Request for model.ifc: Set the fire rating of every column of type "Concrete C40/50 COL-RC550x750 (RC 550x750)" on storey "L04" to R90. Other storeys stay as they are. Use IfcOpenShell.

First a look at what the model holds.

```python
import ifcopenshell
import ifcopenshell.util.element

model = ifcopenshell.open("model.ifc")
print(model.schema)
storey = next(s for s in model.by_type("IfcBuildingStorey") if s.Name == "L04")
columns = [e for e in ifcopenshell.util.element.get_decomposition(storey) if e.is_a("IfcColumn")]
seen = {}
for e in columns:
    element_type = ifcopenshell.util.element.get_type(e)
    key = (element_type.Name if element_type != e and element_type else None, ifcopenshell.util.element.get_pset(e, "Pset_ColumnCommon", "FireRating"))
    seen[key] = seen.get(key, 0) + 1
for (name, value), count in sorted(seen.items(), key=str):
    print(count, "x", name, "|", value)
```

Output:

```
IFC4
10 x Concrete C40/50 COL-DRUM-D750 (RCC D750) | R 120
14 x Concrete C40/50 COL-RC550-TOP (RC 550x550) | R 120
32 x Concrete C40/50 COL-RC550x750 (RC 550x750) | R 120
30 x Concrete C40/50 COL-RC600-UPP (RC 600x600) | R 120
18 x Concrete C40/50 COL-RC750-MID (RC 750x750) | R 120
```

```python
import ifcopenshell
import ifcopenshell.api.pset
import ifcopenshell.util.element

model = ifcopenshell.open("model.ifc")

storey = next(s for s in model.by_type("IfcBuildingStorey") if s.Name == "L04")
columns = [e for e in ifcopenshell.util.element.get_decomposition(storey) if e.is_a("IfcColumn")]

count = 0
for e in columns:
    element_type = ifcopenshell.util.element.get_type(e)
    if element_type in (None, e) or element_type.Name != "Concrete C40/50 COL-RC550x750 (RC 550x750)":
        continue
    # add_pset returns the element's existing set when there is one.
    pset = ifcopenshell.api.pset.add_pset(model, product=e, name="Pset_ColumnCommon")
    ifcopenshell.api.pset.edit_pset(model, pset=pset, properties={"FireRating": "R90"})
    count += 1

print(count, "columns updated")

model.write("model_edited.ifc")
```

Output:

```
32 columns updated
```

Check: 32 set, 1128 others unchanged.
